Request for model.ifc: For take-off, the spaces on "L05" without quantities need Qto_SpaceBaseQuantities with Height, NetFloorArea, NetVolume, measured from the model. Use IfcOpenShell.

First a look at what the model holds.

```python
import ifcopenshell
import ifcopenshell.util.element
import ifcopenshell.util.unit

model = ifcopenshell.open("model.ifc")
print(model.schema)
for unit_type in ("LENGTHUNIT", "AREAUNIT", "VOLUMEUNIT"):
    print(unit_type, ifcopenshell.util.unit.calculate_unit_scale(model, unit_type))
storey = next(s for s in model.by_type("IfcBuildingStorey") if s.Name == "L05")
spaces = [e for e in ifcopenshell.util.element.get_decomposition(storey) if e.is_a("IfcSpace")]
for e in sorted(spaces, key=lambda e: e.id()):
    print(e.id(), e.is_a(), e.Name, list(ifcopenshell.util.element.get_psets(e, qtos_only=True)), sep=" | ")
```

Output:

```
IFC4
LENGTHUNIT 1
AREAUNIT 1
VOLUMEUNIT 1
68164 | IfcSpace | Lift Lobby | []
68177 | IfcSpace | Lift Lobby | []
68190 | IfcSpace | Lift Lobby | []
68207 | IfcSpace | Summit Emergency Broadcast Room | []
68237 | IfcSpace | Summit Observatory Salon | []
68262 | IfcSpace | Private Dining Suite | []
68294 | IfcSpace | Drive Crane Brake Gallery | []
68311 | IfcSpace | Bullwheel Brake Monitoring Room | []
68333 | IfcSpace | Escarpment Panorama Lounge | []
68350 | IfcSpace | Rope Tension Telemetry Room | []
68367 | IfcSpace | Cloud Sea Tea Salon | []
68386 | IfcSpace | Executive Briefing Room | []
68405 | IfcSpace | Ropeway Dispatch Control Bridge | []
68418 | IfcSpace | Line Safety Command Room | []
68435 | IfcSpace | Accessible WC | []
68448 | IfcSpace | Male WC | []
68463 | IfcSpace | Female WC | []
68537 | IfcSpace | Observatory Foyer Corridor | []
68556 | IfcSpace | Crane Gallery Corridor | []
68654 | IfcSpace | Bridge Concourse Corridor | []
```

```python
import ifcopenshell
import ifcopenshell.api.pset
import ifcopenshell.geom
import ifcopenshell.util.element
import ifcopenshell.util.shape
import ifcopenshell.util.unit

model = ifcopenshell.open("model.ifc")
unit_scale = ifcopenshell.util.unit.calculate_unit_scale(model)
area_scale = ifcopenshell.util.unit.calculate_unit_scale(model, "AREAUNIT")
volume_scale = ifcopenshell.util.unit.calculate_unit_scale(model, "VOLUMEUNIT")
settings = ifcopenshell.geom.settings()

storey = next(s for s in model.by_type("IfcBuildingStorey") if s.Name == "L05")
spaces = [e for e in ifcopenshell.util.element.get_decomposition(storey) if e.is_a("IfcSpace")]

for e in sorted(spaces, key=lambda e: e.id()):
    if ifcopenshell.util.element.get_psets(e, qtos_only=True, should_inherit=False):
        continue
    # Geometry comes back in metres, in the element's own axes.
    shape = ifcopenshell.geom.create_shape(settings, e)
    values = {
        "Height": ifcopenshell.util.shape.get_z(shape.geometry) / unit_scale,
        "NetFloorArea": ifcopenshell.util.shape.get_footprint_area(shape.geometry) / area_scale,
        "NetVolume": ifcopenshell.util.shape.get_volume(shape.geometry) / volume_scale,
    }
    qto = ifcopenshell.api.pset.add_qto(model, product=e, name="Qto_SpaceBaseQuantities")
    ifcopenshell.api.pset.edit_qto(model, qto=qto, properties=values)
    print(e.id(), {k: round(v, 3) for k, v in values.items()})

model.write("model-out.ifc")
```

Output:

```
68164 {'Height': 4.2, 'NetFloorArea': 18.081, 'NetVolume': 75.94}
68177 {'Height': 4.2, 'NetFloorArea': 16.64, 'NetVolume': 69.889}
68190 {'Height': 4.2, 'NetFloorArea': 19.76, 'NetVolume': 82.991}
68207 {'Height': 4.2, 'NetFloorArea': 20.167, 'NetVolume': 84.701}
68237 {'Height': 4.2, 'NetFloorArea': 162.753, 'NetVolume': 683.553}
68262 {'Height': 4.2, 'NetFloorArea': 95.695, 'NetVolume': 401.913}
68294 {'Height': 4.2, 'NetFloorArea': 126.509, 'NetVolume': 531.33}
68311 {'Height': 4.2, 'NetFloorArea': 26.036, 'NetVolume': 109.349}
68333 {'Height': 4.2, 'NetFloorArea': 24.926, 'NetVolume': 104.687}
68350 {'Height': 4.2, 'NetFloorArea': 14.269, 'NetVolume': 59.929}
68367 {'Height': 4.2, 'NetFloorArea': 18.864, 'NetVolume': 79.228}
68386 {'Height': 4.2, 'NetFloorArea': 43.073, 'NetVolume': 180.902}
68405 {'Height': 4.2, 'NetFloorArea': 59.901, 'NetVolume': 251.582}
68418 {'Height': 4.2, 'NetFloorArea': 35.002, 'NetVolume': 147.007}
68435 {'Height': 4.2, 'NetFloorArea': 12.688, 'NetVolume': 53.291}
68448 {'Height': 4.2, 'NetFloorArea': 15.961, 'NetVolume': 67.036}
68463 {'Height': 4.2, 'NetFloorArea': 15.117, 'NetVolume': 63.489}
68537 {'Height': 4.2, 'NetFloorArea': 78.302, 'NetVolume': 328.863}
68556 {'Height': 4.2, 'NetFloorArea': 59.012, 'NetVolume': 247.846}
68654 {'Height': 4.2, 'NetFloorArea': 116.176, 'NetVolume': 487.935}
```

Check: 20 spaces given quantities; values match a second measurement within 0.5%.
